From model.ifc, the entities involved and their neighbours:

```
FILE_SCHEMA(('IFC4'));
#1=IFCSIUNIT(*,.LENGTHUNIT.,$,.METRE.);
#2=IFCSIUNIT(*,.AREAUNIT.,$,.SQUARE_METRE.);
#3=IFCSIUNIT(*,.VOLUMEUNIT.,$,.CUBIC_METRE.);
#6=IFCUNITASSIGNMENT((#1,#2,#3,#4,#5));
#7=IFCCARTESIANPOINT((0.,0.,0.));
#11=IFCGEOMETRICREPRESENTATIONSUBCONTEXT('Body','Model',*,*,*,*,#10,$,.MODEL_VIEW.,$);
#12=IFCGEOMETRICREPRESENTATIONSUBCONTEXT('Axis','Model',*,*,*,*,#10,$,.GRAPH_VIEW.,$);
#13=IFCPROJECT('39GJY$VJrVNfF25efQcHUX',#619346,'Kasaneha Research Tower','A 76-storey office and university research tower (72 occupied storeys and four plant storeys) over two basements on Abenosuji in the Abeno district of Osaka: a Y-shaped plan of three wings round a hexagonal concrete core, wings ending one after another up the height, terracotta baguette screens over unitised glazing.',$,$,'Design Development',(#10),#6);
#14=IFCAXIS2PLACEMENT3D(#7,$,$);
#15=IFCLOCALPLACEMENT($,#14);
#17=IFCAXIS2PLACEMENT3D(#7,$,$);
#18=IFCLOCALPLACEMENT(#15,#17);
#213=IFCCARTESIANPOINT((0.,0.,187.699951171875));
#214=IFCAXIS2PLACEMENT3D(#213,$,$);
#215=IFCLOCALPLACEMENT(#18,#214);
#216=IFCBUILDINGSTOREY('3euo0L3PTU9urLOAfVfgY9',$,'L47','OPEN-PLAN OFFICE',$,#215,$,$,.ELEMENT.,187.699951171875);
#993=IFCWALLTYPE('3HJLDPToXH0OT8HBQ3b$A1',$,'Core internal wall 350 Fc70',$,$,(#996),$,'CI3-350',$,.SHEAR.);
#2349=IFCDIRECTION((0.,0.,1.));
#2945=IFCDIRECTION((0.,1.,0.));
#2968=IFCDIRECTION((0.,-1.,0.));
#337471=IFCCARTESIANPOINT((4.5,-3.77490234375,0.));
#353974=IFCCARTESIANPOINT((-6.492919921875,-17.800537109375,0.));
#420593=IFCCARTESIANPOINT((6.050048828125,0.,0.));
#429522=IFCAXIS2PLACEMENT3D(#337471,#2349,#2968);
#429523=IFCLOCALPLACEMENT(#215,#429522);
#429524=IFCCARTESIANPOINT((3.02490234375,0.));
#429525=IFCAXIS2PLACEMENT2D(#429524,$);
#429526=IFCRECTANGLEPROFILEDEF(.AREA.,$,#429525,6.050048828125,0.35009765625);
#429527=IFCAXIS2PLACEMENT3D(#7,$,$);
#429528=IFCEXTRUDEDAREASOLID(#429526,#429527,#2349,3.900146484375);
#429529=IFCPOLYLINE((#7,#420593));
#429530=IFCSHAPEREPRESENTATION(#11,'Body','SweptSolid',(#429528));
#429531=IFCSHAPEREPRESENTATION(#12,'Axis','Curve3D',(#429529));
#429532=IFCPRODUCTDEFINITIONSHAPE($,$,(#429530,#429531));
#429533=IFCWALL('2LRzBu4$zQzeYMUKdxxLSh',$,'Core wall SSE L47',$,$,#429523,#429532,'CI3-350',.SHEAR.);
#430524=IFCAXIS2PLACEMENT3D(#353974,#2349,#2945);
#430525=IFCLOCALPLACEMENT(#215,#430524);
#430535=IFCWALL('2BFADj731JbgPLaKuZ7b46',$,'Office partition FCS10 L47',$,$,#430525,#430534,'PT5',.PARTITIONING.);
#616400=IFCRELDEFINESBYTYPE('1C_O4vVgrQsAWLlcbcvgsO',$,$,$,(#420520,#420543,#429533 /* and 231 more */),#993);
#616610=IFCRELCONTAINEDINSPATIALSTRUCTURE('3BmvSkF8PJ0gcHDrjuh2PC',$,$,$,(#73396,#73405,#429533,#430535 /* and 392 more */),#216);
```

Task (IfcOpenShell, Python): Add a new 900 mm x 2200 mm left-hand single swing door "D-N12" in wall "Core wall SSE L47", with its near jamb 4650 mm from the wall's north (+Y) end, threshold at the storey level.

```python
import numpy as np
import ifcopenshell
import ifcopenshell.api.feature
import ifcopenshell.api.geometry
import ifcopenshell.api.root
import ifcopenshell.api.spatial
import ifcopenshell.geom
import ifcopenshell.util.element
import ifcopenshell.util.placement
import ifcopenshell.util.representation
import ifcopenshell.util.shape
import ifcopenshell.util.unit

model = ifcopenshell.open("model.ifc")
unit_scale = ifcopenshell.util.unit.calculate_unit_scale(model)
settings = ifcopenshell.geom.settings()


def volume(element):
    """Net volume in cubic metres, openings subtracted."""
    shape = ifcopenshell.geom.create_shape(settings, element)
    return ifcopenshell.util.shape.get_volume(shape.geometry)


wall = model.by_guid("2LRzBu4$zQzeYMUKdxxLSh")
storey = ifcopenshell.util.element.get_container(wall, ifc_class="IfcBuildingStorey")
context = ifcopenshell.util.representation.get_context(model, "Model", "Body", "MODEL_VIEW")
before = volume(wall)

width, height, from_end, sill = 0.9, 2.2, 4.65, 0.0  # metres

# The wall runs along its own X axis, and the end named is its -X end.
wall_shape = ifcopenshell.geom.create_shape(settings, wall)
x, y, z = ifcopenshell.util.shape.get_vertices(wall_shape.geometry).T
start = x.min() + from_end
face, thickness = float(y.min()), float(y.max() - y.min())
wall_matrix = ifcopenshell.util.placement.get_local_placement(wall.ObjectPlacement)
level = ifcopenshell.util.placement.get_local_placement(storey.ObjectPlacement)[2, 3]


def in_wall(x, y):
    """Placement at x, y metres in the wall's axes, at sill height."""
    matrix = wall_matrix.copy()
    matrix[:, 3] = wall_matrix @ np.array([x / unit_scale, y / unit_scale, 0.0, 1.0])
    matrix[2, 3] = level + sill / unit_scale
    return matrix


# Opening: a box that overshoots both wall faces by 50 mm.
opening = ifcopenshell.api.root.create_entity(model, ifc_class="IfcOpeningElement", predefined_type="OPENING")
box = ifcopenshell.api.geometry.add_wall_representation(
    model, context=context, length=width, height=height, thickness=thickness + 0.1
)
ifcopenshell.api.geometry.assign_representation(model, product=opening, representation=box)
ifcopenshell.api.geometry.edit_object_placement(model, product=opening, matrix=in_wall(start, face - 0.05), is_si=False)
ifcopenshell.api.feature.add_feature(model, feature=opening, element=wall)

door = ifcopenshell.api.root.create_entity(model, ifc_class="IfcDoor", name="D-N12", predefined_type="DOOR")
door.OverallWidth, door.OverallHeight = width / unit_scale, height / unit_scale
door.OperationType = "SINGLE_SWING_LEFT"
body = ifcopenshell.api.geometry.add_door_representation(
    model,
    context=context,
    overall_width=door.OverallWidth,
    overall_height=door.OverallHeight,
    operation_type="SINGLE_SWING_LEFT",
    lining_properties={"LiningDepth": thickness / unit_scale, "ThresholdDepth": thickness / unit_scale},
)
ifcopenshell.api.geometry.assign_representation(model, product=door, representation=body)
ifcopenshell.api.spatial.assign_container(model, products=[door], relating_structure=storey)
ifcopenshell.api.feature.add_filling(model, opening=opening, element=door)

# The lining spans the wall, so the door starts at the wall face.
ifcopenshell.api.geometry.edit_object_placement(model, product=door, matrix=in_wall(start, face), is_si=False)

after = volume(wall)

print(f"wall volume {before:.3f} -> {after:.3f} m3")

model.write("model_edited.ifc")
```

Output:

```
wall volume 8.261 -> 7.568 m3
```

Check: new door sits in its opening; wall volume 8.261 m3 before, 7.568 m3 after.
